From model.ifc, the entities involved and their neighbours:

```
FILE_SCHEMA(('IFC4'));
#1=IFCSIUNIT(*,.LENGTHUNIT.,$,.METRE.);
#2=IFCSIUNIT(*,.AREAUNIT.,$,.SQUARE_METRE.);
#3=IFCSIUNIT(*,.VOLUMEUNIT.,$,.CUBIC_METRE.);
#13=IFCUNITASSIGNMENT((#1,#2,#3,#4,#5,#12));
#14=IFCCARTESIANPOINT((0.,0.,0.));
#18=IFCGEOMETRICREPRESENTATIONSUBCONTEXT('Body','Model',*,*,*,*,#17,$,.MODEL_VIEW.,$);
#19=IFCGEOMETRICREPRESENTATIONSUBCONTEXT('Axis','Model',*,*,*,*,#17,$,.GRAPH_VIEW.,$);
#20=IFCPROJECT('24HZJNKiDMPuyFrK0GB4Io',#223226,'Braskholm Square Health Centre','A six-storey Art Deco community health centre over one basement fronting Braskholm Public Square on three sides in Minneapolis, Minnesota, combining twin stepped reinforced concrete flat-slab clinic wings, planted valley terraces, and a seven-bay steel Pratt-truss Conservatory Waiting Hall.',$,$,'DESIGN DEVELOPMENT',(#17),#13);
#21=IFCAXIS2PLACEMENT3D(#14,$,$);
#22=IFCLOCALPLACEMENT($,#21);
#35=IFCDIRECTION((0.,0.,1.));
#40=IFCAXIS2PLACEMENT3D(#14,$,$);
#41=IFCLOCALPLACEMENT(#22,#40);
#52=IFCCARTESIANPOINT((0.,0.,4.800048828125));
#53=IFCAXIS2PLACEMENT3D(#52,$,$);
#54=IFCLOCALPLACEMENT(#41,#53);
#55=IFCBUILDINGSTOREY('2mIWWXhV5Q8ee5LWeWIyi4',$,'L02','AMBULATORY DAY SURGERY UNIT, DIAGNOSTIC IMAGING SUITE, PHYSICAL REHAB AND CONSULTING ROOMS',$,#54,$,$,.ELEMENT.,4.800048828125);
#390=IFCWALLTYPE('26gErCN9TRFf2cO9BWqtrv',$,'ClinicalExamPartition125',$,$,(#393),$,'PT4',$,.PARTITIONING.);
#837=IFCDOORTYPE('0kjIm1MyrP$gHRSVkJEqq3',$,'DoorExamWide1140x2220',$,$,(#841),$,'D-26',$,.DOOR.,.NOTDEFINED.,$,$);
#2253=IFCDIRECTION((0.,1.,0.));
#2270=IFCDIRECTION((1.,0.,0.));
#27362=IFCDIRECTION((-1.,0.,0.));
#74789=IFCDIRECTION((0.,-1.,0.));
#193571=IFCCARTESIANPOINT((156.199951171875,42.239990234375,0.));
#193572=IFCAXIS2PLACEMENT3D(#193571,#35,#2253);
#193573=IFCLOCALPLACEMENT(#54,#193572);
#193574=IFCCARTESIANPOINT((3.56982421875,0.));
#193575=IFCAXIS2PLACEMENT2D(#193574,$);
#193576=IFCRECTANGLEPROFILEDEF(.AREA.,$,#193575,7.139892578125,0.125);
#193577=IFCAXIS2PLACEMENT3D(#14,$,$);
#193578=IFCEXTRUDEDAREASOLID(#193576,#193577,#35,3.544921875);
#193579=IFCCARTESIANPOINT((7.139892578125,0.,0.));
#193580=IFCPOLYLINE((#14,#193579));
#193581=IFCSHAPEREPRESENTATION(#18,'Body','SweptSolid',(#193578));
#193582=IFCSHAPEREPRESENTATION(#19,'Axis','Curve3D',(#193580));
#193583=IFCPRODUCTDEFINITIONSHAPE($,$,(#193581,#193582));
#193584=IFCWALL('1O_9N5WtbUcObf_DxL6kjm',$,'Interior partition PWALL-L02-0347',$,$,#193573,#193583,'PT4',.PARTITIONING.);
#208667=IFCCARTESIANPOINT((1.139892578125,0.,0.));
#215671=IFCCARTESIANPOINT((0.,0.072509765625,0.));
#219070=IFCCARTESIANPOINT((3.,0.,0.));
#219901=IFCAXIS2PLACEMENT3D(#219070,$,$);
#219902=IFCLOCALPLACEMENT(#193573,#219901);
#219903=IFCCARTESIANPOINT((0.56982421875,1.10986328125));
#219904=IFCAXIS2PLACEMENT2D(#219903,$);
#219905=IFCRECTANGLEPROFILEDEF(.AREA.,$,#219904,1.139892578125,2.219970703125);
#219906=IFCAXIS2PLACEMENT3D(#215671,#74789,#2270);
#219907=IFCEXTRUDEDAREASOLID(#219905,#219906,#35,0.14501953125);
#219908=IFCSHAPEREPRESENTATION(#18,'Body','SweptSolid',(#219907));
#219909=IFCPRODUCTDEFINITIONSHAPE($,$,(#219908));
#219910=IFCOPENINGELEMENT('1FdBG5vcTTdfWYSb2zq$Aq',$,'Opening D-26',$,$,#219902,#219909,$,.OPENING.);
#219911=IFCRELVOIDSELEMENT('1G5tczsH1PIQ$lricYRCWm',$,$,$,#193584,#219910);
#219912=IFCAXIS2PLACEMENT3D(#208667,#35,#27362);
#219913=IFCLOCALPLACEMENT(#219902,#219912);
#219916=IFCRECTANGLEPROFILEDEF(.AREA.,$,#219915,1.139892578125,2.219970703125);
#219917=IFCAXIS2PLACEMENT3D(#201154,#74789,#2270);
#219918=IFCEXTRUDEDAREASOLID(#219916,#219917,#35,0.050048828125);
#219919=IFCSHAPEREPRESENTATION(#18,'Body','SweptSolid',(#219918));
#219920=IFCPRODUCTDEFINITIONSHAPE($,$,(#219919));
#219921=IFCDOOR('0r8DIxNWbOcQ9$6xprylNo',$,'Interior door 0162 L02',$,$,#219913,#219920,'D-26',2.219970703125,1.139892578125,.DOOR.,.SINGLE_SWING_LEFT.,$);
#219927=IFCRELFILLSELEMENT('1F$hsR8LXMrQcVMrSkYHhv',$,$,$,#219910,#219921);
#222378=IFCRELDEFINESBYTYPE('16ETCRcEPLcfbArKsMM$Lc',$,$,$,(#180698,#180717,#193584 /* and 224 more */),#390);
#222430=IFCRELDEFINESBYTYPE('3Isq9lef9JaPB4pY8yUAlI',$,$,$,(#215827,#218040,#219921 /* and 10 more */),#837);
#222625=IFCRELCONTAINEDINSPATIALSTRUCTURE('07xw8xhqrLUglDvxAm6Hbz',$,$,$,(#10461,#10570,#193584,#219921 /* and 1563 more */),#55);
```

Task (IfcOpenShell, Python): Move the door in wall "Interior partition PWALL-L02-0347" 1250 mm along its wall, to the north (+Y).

```python
import ifcopenshell
import ifcopenshell.api.geometry
import ifcopenshell.util.placement

model = ifcopenshell.open("model.ifc")

door = model.by_id(219921)
opening = door.FillsVoids[0].RelatingOpeningElement
wall = opening.VoidsElements[0].RelatingBuildingElement

wall_matrix = ifcopenshell.util.placement.get_local_placement(wall.ObjectPlacement)
shift = wall_matrix[:3, 0] * 1.25
before = ifcopenshell.util.placement.get_local_placement(door.ObjectPlacement)[:3, 3].copy()

# The door is placed relative to its opening, so it follows when the opening moves.
matrix = ifcopenshell.util.placement.get_local_placement(opening.ObjectPlacement)
matrix[:3, 3] += shift
ifcopenshell.api.geometry.edit_object_placement(
    model, product=opening, matrix=matrix, is_si=False, should_transform_children=True
)

after = ifcopenshell.util.placement.get_local_placement(door.ObjectPlacement)[:3, 3]
print("door moved by", (after - before).round(3) + 0.0)

model.write("model_edited.ifc")
```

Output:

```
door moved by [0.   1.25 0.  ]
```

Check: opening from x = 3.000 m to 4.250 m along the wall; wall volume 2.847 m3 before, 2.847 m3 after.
